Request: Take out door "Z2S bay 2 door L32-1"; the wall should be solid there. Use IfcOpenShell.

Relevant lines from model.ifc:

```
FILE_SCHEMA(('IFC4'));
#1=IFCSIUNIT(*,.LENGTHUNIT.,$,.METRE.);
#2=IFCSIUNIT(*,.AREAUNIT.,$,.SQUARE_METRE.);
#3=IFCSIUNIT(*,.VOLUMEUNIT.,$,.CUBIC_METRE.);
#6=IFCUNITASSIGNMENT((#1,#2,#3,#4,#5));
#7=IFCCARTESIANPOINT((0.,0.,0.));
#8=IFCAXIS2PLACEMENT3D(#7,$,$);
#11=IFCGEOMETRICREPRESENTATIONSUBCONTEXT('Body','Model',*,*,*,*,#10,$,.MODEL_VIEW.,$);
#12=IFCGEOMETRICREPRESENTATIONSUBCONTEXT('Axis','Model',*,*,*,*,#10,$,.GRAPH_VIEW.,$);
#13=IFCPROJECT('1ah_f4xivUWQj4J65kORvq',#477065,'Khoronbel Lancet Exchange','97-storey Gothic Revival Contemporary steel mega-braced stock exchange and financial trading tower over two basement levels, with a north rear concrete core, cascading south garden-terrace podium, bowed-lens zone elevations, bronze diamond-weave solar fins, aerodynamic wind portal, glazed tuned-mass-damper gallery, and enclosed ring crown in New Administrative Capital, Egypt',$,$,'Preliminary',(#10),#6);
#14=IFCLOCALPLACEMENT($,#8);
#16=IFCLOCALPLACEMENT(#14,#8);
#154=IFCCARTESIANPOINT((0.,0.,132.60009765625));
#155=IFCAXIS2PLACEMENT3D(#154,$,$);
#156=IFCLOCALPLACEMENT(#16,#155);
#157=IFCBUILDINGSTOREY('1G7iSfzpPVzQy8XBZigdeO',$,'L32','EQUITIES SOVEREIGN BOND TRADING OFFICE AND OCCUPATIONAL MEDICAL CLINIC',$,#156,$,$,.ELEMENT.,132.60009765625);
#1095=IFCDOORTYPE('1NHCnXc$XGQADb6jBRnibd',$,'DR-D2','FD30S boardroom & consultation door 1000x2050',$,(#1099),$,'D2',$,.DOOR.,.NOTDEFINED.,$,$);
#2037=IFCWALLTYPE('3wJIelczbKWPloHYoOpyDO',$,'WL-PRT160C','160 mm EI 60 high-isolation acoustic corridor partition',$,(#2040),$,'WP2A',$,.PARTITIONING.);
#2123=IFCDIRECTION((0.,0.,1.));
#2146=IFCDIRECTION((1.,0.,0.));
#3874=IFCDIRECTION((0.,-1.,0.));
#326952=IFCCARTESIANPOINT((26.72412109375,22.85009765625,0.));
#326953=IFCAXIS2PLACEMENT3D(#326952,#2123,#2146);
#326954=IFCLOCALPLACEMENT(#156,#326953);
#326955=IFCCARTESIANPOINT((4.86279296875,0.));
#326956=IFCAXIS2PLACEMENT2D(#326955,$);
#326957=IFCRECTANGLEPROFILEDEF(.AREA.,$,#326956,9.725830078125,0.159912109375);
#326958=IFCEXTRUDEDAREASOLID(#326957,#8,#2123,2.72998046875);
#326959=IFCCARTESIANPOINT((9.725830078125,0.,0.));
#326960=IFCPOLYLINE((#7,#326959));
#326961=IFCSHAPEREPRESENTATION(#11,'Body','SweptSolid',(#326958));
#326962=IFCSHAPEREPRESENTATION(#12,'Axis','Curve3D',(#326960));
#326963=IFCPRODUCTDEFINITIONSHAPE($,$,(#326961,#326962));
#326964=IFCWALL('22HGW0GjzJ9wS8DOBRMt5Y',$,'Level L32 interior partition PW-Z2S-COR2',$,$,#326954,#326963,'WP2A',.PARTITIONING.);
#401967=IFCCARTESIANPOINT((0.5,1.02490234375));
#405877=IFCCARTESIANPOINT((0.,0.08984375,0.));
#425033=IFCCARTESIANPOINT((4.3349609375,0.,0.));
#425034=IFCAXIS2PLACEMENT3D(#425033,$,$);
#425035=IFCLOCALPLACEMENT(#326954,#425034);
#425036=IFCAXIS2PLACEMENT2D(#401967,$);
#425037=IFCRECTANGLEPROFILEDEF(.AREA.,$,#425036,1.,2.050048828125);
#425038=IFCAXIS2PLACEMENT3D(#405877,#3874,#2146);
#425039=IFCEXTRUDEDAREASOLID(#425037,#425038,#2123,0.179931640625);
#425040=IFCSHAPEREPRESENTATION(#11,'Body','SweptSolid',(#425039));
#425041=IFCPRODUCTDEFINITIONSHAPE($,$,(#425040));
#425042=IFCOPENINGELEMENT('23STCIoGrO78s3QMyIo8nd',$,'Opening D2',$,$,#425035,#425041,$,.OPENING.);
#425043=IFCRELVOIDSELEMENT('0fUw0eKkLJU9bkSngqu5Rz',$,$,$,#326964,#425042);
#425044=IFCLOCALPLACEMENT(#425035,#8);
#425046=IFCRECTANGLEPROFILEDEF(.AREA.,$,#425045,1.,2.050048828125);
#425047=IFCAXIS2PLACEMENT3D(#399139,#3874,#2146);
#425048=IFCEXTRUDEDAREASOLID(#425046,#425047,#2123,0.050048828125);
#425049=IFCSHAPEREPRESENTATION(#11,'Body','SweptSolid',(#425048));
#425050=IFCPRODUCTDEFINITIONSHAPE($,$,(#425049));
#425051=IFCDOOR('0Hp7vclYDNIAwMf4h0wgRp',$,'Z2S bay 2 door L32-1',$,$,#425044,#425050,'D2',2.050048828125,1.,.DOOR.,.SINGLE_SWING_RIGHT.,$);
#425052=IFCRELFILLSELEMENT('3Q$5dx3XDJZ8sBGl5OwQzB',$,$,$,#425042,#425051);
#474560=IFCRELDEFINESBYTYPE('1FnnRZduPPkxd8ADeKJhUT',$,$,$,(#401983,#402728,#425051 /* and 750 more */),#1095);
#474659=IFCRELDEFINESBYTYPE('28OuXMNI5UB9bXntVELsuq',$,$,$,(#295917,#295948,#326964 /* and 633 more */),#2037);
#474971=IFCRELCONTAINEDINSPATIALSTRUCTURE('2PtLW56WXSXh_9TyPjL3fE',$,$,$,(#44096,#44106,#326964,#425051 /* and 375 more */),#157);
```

```python
import ifcopenshell
import ifcopenshell.api.feature
import ifcopenshell.api.root
import ifcopenshell.geom
import ifcopenshell.util.shape

model = ifcopenshell.open("model.ifc")
settings = ifcopenshell.geom.settings()


def volume(element):
    """Net volume in cubic metres, openings subtracted."""
    shape = ifcopenshell.geom.create_shape(settings, element)
    return ifcopenshell.util.shape.get_volume(shape.geometry)


door = model.by_guid("0Hp7vclYDNIAwMf4h0wgRp")
opening = door.FillsVoids[0].RelatingOpeningElement
wall = opening.VoidsElements[0].RelatingBuildingElement
before = volume(wall)

ifcopenshell.api.root.remove_product(model, product=door)
ifcopenshell.api.feature.remove_feature(model, feature=opening)

after = volume(wall)

print(f"wall volume {before:.3f} -> {after:.3f} m3")

model.write("model-out.ifc")
```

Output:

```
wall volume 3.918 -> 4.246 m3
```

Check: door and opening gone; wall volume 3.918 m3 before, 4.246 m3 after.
